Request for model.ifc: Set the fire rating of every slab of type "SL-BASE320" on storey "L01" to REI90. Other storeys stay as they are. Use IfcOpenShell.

First a look at what the model holds.

```python
import ifcopenshell
import ifcopenshell.util.element

model = ifcopenshell.open("model.ifc")
print(model.schema)
storey = next(s for s in model.by_type("IfcBuildingStorey") if s.Name == "L01")
slabs = [e for e in ifcopenshell.util.element.get_decomposition(storey) if e.is_a("IfcSlab")]
seen = {}
for e in slabs:
    element_type = ifcopenshell.util.element.get_type(e)
    key = (element_type.Name if element_type != e and element_type else None, ifcopenshell.util.element.get_pset(e, "Pset_SlabCommon", "FireRating"))
    seen[key] = seen.get(key, 0) + 1
for (name, value), count in sorted(seen.items(), key=str):
    print(count, "x", name, "|", value)
```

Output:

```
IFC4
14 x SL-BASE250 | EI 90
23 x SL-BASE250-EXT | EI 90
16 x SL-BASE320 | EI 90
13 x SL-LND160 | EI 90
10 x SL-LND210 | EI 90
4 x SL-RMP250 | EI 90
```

```python
import ifcopenshell
import ifcopenshell.api.pset
import ifcopenshell.util.element

model = ifcopenshell.open("model.ifc")

storey = next(s for s in model.by_type("IfcBuildingStorey") if s.Name == "L01")
slabs = [e for e in ifcopenshell.util.element.get_decomposition(storey) if e.is_a("IfcSlab")]

count = 0
for e in slabs:
    element_type = ifcopenshell.util.element.get_type(e)
    if element_type in (None, e) or element_type.Name != "SL-BASE320":
        continue
    # add_pset returns the element's existing set when there is one.
    pset = ifcopenshell.api.pset.add_pset(model, product=e, name="Pset_SlabCommon")
    ifcopenshell.api.pset.edit_pset(model, pset=pset, properties={"FireRating": "REI90"})
    count += 1

print(count, "slabs updated")

model.write("model_v2.ifc")
```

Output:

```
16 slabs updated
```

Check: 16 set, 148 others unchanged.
